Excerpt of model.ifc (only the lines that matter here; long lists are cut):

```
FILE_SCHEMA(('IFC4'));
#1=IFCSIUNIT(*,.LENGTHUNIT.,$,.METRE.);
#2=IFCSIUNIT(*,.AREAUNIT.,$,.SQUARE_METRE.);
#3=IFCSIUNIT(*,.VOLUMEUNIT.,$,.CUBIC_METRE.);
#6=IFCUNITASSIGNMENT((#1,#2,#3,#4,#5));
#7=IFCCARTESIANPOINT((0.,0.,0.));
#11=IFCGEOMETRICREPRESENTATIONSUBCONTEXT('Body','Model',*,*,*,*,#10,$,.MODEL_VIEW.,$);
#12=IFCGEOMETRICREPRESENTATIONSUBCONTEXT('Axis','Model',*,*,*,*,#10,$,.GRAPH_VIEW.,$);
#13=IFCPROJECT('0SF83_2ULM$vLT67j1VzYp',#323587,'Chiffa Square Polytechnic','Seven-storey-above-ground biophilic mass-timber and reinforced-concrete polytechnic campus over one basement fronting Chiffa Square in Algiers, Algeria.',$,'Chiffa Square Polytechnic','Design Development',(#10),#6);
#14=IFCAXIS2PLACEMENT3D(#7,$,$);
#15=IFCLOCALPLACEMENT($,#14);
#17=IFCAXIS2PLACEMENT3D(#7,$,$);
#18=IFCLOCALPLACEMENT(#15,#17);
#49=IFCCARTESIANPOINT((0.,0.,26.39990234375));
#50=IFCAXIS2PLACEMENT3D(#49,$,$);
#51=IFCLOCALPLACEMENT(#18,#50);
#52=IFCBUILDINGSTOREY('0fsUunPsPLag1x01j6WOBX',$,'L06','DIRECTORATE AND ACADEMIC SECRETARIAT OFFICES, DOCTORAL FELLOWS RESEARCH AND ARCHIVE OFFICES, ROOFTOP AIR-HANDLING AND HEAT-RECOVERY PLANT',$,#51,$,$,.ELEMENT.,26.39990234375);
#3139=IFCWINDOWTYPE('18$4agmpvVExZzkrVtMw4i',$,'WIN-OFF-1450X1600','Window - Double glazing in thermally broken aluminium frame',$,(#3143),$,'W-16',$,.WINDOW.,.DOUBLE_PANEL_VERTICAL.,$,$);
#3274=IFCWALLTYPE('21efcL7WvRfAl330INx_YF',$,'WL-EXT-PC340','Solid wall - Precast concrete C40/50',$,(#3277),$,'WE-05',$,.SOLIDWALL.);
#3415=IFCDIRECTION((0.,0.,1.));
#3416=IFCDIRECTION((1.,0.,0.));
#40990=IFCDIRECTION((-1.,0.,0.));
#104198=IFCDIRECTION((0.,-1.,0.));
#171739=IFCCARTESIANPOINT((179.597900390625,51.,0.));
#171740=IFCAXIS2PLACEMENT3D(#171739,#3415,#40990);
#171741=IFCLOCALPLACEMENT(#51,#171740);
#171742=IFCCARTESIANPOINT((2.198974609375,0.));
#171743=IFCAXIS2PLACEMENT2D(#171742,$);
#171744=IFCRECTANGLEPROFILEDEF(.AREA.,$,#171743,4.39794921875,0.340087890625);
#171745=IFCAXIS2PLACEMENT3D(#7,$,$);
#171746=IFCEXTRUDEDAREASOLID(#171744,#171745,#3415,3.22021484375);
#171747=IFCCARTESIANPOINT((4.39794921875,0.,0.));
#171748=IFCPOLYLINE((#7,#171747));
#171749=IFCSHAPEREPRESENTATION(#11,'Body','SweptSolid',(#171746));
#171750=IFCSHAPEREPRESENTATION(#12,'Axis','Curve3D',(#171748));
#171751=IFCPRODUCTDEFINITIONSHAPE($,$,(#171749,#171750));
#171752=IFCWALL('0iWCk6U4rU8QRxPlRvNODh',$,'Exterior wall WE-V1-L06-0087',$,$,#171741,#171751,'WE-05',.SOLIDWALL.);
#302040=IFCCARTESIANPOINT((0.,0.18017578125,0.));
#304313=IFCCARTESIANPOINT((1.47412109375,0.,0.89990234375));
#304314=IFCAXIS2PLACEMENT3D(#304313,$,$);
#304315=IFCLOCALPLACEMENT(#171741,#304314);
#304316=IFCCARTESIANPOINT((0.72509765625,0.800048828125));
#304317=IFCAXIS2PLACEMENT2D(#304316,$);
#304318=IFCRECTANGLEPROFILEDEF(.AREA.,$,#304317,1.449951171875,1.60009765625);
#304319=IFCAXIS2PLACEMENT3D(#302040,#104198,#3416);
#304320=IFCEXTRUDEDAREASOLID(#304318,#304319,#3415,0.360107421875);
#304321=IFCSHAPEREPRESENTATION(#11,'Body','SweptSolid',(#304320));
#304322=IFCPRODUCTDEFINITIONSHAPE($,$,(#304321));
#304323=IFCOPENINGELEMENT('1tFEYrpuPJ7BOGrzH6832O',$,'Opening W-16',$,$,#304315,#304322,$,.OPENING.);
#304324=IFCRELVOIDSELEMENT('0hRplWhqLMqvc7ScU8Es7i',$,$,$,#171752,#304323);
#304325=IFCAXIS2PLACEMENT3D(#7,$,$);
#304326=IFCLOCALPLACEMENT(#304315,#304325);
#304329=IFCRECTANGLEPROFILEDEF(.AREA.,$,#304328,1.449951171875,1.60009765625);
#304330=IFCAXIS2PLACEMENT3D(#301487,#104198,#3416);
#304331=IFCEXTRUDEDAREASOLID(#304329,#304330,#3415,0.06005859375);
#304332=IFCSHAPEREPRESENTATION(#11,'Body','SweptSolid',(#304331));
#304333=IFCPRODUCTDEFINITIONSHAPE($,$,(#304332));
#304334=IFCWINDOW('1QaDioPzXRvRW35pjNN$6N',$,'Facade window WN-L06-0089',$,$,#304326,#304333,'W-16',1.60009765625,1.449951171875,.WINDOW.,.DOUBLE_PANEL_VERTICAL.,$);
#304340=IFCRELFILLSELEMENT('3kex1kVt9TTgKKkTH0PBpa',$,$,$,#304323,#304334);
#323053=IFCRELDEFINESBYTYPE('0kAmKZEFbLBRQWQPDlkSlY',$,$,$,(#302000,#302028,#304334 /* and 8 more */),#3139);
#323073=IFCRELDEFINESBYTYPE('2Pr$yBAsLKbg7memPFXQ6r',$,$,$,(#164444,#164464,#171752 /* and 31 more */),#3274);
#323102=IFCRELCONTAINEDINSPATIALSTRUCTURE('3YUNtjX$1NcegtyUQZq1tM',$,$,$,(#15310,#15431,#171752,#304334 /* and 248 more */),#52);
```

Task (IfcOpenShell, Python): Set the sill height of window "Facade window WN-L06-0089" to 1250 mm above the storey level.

```python
import numpy as np
import ifcopenshell
import ifcopenshell.api.geometry
import ifcopenshell.geom
import ifcopenshell.util.element
import ifcopenshell.util.placement
import ifcopenshell.util.shape
import ifcopenshell.util.unit

model = ifcopenshell.open("model.ifc")
unit_scale = ifcopenshell.util.unit.calculate_unit_scale(model)

window = model.by_guid("1QaDioPzXRvRW35pjNN$6N")
opening = window.FillsVoids[0].RelatingOpeningElement
storey = ifcopenshell.util.element.get_container(window, ifc_class="IfcBuildingStorey")
level = ifcopenshell.util.placement.get_local_placement(storey.ObjectPlacement)[2, 3]

# The opening's origin need not be at the sill, so measure its lowest point.
shape = ifcopenshell.geom.create_shape(ifcopenshell.geom.settings(), opening)
bottom = ifcopenshell.util.shape.get_shape_bottom_elevation(shape, shape.geometry) / unit_scale
dz = level + 1.25 / unit_scale - bottom

shift = np.array([0.0, 0.0, dz])
# The window is placed relative to its opening, so it follows when the opening moves.
matrix = ifcopenshell.util.placement.get_local_placement(opening.ObjectPlacement)
matrix[:3, 3] += shift
ifcopenshell.api.geometry.edit_object_placement(
    model, product=opening, matrix=matrix, is_si=False, should_transform_children=True
)

print(f"moved by {dz * unit_scale:+.3f} m")

model.write("model_rev.ifc")
```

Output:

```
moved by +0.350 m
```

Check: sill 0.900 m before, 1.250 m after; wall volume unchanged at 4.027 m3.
